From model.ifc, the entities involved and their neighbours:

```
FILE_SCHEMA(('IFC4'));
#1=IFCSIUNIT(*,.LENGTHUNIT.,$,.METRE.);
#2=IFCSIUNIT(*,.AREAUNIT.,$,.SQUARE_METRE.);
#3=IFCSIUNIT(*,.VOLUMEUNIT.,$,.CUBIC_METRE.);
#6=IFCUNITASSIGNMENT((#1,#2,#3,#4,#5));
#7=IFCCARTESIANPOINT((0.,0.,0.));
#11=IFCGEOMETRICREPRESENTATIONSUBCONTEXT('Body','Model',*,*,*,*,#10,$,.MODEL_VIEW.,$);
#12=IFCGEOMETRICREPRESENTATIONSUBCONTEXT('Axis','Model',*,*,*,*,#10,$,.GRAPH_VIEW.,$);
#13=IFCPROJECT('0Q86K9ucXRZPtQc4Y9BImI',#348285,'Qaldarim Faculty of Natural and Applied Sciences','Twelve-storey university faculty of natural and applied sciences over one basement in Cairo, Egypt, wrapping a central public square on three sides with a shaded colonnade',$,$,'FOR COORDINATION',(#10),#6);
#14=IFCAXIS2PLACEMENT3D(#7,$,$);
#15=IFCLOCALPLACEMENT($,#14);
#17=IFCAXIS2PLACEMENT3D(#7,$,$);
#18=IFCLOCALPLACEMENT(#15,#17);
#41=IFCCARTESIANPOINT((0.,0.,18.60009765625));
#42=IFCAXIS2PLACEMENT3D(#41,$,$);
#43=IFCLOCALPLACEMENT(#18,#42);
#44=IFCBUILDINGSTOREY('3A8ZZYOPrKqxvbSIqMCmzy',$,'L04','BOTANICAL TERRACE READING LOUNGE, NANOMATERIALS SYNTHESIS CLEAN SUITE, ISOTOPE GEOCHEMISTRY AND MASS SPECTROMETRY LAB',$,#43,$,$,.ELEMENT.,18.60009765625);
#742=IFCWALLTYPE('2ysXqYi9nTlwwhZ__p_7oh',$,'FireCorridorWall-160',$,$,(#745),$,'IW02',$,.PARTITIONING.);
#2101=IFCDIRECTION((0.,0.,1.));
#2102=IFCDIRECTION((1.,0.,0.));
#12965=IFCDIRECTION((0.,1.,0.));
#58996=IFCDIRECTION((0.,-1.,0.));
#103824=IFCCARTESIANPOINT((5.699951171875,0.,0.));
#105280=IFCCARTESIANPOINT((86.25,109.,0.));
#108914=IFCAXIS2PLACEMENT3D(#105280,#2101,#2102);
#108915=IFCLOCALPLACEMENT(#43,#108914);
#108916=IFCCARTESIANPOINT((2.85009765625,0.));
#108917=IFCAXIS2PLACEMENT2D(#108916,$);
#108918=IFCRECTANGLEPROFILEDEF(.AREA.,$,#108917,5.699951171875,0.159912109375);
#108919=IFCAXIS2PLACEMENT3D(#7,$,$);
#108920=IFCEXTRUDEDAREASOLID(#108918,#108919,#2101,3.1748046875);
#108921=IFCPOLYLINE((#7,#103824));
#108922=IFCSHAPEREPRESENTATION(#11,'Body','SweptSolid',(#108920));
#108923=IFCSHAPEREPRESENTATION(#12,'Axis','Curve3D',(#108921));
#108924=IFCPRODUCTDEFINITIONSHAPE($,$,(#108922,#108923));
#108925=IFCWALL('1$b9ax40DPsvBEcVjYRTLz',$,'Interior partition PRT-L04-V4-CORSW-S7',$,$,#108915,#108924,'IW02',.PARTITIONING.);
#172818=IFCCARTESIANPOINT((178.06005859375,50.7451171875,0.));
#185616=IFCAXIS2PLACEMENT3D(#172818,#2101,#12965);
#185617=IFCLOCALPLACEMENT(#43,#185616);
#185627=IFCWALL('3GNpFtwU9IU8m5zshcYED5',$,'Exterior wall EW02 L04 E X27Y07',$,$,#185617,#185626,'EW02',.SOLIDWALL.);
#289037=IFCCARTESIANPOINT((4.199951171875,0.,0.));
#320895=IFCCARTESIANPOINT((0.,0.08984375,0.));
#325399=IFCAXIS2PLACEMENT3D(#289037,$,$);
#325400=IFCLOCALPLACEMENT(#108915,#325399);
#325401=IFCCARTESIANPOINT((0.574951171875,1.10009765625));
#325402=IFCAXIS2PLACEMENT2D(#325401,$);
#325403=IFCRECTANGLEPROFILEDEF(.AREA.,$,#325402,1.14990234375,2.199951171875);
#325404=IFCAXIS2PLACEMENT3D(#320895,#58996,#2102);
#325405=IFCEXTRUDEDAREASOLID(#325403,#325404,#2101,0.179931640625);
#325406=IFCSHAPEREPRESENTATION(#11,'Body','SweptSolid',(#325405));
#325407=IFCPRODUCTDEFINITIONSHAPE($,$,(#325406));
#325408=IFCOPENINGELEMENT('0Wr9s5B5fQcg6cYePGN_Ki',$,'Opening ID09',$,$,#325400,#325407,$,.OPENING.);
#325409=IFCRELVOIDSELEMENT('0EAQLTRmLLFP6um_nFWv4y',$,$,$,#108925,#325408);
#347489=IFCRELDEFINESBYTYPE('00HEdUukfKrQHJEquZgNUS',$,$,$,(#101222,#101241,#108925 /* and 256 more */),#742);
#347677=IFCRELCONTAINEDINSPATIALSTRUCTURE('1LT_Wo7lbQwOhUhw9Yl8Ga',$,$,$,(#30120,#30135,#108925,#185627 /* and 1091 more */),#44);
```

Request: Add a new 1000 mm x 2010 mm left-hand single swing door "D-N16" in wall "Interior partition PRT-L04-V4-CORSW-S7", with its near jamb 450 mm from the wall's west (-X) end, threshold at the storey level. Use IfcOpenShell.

```python
import numpy as np
import ifcopenshell
import ifcopenshell.api.feature
import ifcopenshell.api.geometry
import ifcopenshell.api.root
import ifcopenshell.api.spatial
import ifcopenshell.geom
import ifcopenshell.util.element
import ifcopenshell.util.placement
import ifcopenshell.util.representation
import ifcopenshell.util.shape
import ifcopenshell.util.unit

model = ifcopenshell.open("model.ifc")
unit_scale = ifcopenshell.util.unit.calculate_unit_scale(model)
settings = ifcopenshell.geom.settings()


def volume(element):
    """Net volume in cubic metres, openings subtracted."""
    shape = ifcopenshell.geom.create_shape(settings, element)
    return ifcopenshell.util.shape.get_volume(shape.geometry)


wall = model.by_guid("1$b9ax40DPsvBEcVjYRTLz")
storey = ifcopenshell.util.element.get_container(wall, ifc_class="IfcBuildingStorey")
context = ifcopenshell.util.representation.get_context(model, "Model", "Body", "MODEL_VIEW")
before = volume(wall)

width, height, from_end, sill = 1, 2.01, 0.45, 0.0  # metres

# The wall runs along its own X axis, and the end named is its -X end.
wall_shape = ifcopenshell.geom.create_shape(settings, wall)
x, y, z = ifcopenshell.util.shape.get_vertices(wall_shape.geometry).T
start = x.min() + from_end
face, thickness = float(y.min()), float(y.max() - y.min())
wall_matrix = ifcopenshell.util.placement.get_local_placement(wall.ObjectPlacement)
level = ifcopenshell.util.placement.get_local_placement(storey.ObjectPlacement)[2, 3]


def in_wall(x, y):
    """Placement at x, y metres in the wall's axes, at sill height."""
    matrix = wall_matrix.copy()
    matrix[:, 3] = wall_matrix @ np.array([x / unit_scale, y / unit_scale, 0.0, 1.0])
    matrix[2, 3] = level + sill / unit_scale
    return matrix


# Opening: a box that overshoots both wall faces by 50 mm.
opening = ifcopenshell.api.root.create_entity(model, ifc_class="IfcOpeningElement", predefined_type="OPENING")
box = ifcopenshell.api.geometry.add_wall_representation(
    model, context=context, length=width, height=height, thickness=thickness + 0.1
)
ifcopenshell.api.geometry.assign_representation(model, product=opening, representation=box)
ifcopenshell.api.geometry.edit_object_placement(model, product=opening, matrix=in_wall(start, face - 0.05), is_si=False)
ifcopenshell.api.feature.add_feature(model, feature=opening, element=wall)

door = ifcopenshell.api.root.create_entity(model, ifc_class="IfcDoor", name="D-N16", predefined_type="DOOR")
door.OverallWidth, door.OverallHeight = width / unit_scale, height / unit_scale
door.OperationType = "SINGLE_SWING_LEFT"
body = ifcopenshell.api.geometry.add_door_representation(
    model,
    context=context,
    overall_width=door.OverallWidth,
    overall_height=door.OverallHeight,
    operation_type="SINGLE_SWING_LEFT",
    lining_properties={"LiningDepth": thickness / unit_scale, "ThresholdDepth": thickness / unit_scale},
)
ifcopenshell.api.geometry.assign_representation(model, product=door, representation=body)
ifcopenshell.api.spatial.assign_container(model, products=[door], relating_structure=storey)
ifcopenshell.api.feature.add_filling(model, opening=opening, element=door)

# The lining spans the wall, so the door starts at the wall face.
ifcopenshell.api.geometry.edit_object_placement(model, product=door, matrix=in_wall(start, face), is_si=False)

after = volume(wall)

print(f"wall volume {before:.3f} -> {after:.3f} m3")

model.write("model_v2.ifc")
```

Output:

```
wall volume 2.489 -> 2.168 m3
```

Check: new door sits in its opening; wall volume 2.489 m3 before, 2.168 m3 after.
